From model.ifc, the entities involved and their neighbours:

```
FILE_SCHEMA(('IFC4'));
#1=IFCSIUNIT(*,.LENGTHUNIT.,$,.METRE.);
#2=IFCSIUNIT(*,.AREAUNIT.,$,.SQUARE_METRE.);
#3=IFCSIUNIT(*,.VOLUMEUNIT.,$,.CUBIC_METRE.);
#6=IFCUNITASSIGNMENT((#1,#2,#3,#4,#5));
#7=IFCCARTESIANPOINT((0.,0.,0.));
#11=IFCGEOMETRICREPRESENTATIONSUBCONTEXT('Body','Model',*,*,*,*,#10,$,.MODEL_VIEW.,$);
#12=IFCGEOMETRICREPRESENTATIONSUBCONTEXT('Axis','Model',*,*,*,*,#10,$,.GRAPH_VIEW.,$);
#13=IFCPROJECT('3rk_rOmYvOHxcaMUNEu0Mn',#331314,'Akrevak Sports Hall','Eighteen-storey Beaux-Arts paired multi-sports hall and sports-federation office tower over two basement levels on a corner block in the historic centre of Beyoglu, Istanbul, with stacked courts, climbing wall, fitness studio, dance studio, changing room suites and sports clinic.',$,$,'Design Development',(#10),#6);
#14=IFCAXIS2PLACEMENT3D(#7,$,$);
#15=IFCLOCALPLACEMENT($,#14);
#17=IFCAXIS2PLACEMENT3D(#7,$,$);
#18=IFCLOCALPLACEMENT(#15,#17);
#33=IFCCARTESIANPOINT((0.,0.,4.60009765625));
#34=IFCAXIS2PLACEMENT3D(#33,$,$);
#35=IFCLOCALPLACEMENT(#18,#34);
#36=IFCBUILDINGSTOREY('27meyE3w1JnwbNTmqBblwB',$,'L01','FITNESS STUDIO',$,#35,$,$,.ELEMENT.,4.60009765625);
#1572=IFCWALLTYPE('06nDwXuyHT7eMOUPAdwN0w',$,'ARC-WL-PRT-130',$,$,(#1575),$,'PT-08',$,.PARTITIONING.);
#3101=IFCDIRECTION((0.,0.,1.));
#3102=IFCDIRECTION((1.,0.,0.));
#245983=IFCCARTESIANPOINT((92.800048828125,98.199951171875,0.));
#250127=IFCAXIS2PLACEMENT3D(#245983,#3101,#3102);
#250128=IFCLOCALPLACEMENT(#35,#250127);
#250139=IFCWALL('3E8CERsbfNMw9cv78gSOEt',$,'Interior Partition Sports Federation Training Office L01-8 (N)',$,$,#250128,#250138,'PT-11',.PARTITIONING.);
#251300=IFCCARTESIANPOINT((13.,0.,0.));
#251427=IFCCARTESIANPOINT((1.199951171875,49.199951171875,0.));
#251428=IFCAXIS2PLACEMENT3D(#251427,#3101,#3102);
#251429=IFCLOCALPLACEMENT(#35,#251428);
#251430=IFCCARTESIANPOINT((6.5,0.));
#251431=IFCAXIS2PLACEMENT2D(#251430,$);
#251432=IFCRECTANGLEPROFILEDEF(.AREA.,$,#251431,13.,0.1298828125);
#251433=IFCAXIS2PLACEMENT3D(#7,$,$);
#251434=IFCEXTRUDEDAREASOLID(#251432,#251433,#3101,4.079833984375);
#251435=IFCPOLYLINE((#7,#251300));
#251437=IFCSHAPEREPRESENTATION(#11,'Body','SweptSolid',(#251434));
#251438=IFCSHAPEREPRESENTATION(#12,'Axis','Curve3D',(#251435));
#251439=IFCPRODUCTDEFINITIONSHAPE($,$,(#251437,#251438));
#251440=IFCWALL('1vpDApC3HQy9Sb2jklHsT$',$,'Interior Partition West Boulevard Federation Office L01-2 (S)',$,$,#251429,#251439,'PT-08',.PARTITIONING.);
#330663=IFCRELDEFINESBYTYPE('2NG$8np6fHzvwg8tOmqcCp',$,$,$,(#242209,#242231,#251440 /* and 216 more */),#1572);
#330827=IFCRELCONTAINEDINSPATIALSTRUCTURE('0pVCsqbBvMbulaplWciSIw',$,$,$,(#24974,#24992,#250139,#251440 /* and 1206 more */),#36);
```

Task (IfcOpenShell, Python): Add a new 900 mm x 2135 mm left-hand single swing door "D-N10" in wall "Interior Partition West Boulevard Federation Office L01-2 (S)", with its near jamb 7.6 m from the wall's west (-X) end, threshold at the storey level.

```python
import numpy as np
import ifcopenshell
import ifcopenshell.api.feature
import ifcopenshell.api.geometry
import ifcopenshell.api.root
import ifcopenshell.api.spatial
import ifcopenshell.geom
import ifcopenshell.util.element
import ifcopenshell.util.placement
import ifcopenshell.util.representation
import ifcopenshell.util.shape
import ifcopenshell.util.unit

model = ifcopenshell.open("model.ifc")
unit_scale = ifcopenshell.util.unit.calculate_unit_scale(model)
settings = ifcopenshell.geom.settings()


def volume(element):
    """Net volume in cubic metres, openings subtracted."""
    shape = ifcopenshell.geom.create_shape(settings, element)
    return ifcopenshell.util.shape.get_volume(shape.geometry)


wall = model.by_guid("1vpDApC3HQy9Sb2jklHsT$")
storey = ifcopenshell.util.element.get_container(wall, ifc_class="IfcBuildingStorey")
context = ifcopenshell.util.representation.get_context(model, "Model", "Body", "MODEL_VIEW")
before = volume(wall)

width, height, from_end, sill = 0.9, 2.135, 7.6, 0.0  # metres

# The wall runs along its own X axis, and the end named is its -X end.
wall_shape = ifcopenshell.geom.create_shape(settings, wall)
x, y, z = ifcopenshell.util.shape.get_vertices(wall_shape.geometry).T
start = x.min() + from_end
face, thickness = float(y.min()), float(y.max() - y.min())
wall_matrix = ifcopenshell.util.placement.get_local_placement(wall.ObjectPlacement)
level = ifcopenshell.util.placement.get_local_placement(storey.ObjectPlacement)[2, 3]


def in_wall(x, y):
    """Placement at x, y metres in the wall's axes, at sill height."""
    matrix = wall_matrix.copy()
    matrix[:, 3] = wall_matrix @ np.array([x / unit_scale, y / unit_scale, 0.0, 1.0])
    matrix[2, 3] = level + sill / unit_scale
    return matrix


# Opening: a box that overshoots both wall faces by 50 mm.
opening = ifcopenshell.api.root.create_entity(model, ifc_class="IfcOpeningElement", predefined_type="OPENING")
box = ifcopenshell.api.geometry.add_wall_representation(
    model, context=context, length=width, height=height, thickness=thickness + 0.1
)
ifcopenshell.api.geometry.assign_representation(model, product=opening, representation=box)
ifcopenshell.api.geometry.edit_object_placement(model, product=opening, matrix=in_wall(start, face - 0.05), is_si=False)
ifcopenshell.api.feature.add_feature(model, feature=opening, element=wall)

door = ifcopenshell.api.root.create_entity(model, ifc_class="IfcDoor", name="D-N10", predefined_type="DOOR")
door.OverallWidth, door.OverallHeight = width / unit_scale, height / unit_scale
door.OperationType = "SINGLE_SWING_LEFT"
body = ifcopenshell.api.geometry.add_door_representation(
    model,
    context=context,
    overall_width=door.OverallWidth,
    overall_height=door.OverallHeight,
    operation_type="SINGLE_SWING_LEFT",
    lining_properties={"LiningDepth": thickness / unit_scale, "ThresholdDepth": thickness / unit_scale},
)
ifcopenshell.api.geometry.assign_representation(model, product=door, representation=body)
ifcopenshell.api.spatial.assign_container(model, products=[door], relating_structure=storey)
ifcopenshell.api.feature.add_filling(model, opening=opening, element=door)

# The lining spans the wall, so the door starts at the wall face.
ifcopenshell.api.geometry.edit_object_placement(model, product=door, matrix=in_wall(start, face), is_si=False)

after = volume(wall)

print(f"wall volume {before:.3f} -> {after:.3f} m3")

model.write("model_edited.ifc")
```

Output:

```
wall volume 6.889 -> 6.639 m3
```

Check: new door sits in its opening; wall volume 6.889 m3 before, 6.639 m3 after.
